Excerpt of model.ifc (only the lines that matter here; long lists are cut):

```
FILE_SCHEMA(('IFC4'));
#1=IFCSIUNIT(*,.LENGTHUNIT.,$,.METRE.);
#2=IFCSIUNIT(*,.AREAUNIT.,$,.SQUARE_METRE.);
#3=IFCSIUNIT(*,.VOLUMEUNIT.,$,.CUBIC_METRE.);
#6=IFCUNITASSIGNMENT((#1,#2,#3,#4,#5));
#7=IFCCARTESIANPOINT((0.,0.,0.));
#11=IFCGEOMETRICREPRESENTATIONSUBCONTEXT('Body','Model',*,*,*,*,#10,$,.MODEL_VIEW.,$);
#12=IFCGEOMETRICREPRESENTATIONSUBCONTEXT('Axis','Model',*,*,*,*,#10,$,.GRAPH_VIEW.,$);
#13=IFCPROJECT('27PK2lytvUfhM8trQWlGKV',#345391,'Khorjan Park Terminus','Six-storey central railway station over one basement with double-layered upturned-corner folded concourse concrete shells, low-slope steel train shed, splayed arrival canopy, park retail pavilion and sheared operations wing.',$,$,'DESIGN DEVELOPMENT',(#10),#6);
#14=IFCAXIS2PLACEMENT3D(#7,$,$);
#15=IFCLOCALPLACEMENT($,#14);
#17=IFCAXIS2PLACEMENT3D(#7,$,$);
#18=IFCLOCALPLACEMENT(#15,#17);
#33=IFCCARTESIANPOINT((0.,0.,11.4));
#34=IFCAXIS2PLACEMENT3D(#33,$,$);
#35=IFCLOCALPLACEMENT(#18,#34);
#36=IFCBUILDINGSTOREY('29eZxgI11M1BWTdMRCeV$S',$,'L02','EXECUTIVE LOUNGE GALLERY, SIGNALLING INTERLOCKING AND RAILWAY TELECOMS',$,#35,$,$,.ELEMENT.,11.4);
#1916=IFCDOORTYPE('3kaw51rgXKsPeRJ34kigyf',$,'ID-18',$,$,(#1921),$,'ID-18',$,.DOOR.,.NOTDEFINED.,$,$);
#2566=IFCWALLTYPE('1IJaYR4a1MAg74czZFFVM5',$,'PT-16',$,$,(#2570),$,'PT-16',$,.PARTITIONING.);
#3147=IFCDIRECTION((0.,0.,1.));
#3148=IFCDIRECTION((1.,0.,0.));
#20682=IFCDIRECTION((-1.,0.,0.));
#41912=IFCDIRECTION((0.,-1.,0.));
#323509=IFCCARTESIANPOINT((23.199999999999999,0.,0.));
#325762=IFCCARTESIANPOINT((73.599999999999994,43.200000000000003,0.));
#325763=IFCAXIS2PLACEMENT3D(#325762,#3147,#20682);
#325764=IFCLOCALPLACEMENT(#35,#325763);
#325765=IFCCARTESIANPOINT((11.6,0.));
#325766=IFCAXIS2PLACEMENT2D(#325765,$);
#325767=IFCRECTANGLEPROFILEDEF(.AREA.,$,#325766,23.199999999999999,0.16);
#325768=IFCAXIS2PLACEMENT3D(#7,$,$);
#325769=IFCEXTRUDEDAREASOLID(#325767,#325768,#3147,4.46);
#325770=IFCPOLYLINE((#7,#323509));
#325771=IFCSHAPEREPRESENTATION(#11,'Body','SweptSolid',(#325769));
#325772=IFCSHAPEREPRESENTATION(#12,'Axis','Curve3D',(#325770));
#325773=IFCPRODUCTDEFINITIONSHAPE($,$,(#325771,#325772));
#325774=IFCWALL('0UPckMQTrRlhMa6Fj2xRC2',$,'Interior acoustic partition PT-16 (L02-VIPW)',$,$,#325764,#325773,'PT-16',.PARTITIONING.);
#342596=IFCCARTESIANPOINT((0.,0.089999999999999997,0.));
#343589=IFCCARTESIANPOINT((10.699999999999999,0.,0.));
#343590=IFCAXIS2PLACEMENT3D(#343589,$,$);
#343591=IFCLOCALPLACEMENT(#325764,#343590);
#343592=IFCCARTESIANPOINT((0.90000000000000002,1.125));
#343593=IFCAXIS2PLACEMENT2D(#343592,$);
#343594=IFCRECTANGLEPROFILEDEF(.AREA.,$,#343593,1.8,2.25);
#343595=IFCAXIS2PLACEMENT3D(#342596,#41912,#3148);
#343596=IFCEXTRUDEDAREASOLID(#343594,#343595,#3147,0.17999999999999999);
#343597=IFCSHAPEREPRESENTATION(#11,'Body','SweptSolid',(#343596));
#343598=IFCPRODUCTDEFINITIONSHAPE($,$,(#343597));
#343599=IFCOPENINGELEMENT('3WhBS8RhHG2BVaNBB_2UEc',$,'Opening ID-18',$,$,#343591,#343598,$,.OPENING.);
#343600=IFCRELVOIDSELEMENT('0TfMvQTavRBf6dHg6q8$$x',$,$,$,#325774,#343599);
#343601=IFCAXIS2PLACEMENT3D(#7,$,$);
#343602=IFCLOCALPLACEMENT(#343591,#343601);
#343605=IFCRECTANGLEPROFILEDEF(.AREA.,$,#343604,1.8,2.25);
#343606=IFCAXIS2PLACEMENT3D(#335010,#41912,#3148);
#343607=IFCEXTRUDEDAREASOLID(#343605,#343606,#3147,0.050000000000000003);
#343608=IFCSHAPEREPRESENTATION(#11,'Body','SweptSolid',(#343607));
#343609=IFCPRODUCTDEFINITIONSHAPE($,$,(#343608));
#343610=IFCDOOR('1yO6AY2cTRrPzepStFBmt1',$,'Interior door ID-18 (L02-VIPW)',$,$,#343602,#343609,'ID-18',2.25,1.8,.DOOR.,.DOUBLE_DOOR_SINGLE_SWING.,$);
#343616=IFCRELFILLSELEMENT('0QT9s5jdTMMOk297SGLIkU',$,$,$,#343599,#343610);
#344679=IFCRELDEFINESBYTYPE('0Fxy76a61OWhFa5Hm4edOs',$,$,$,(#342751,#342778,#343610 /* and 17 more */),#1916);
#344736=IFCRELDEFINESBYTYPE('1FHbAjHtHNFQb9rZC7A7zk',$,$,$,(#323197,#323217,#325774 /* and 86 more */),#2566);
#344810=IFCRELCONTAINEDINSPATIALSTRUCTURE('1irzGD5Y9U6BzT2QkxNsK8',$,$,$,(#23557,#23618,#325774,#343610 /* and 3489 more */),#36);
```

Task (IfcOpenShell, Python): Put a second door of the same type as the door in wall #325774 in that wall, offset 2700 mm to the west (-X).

```python
import ifcopenshell
import ifcopenshell.api.feature
import ifcopenshell.api.geometry
import ifcopenshell.api.root
import ifcopenshell.geom
import ifcopenshell.util.element
import ifcopenshell.util.placement
import ifcopenshell.util.shape
import ifcopenshell.util.unit

model = ifcopenshell.open("model.ifc")
unit_scale = ifcopenshell.util.unit.calculate_unit_scale(model)
settings = ifcopenshell.geom.settings()


def volume(element):
    """Net volume in cubic metres, openings subtracted."""
    shape = ifcopenshell.geom.create_shape(settings, element)
    return ifcopenshell.util.shape.get_volume(shape.geometry)


door = model.by_guid("1yO6AY2cTRrPzepStFBmt1")
opening = door.FillsVoids[0].RelatingOpeningElement
wall = opening.VoidsElements[0].RelatingBuildingElement
before = volume(wall)
shift = ifcopenshell.util.placement.get_local_placement(wall.ObjectPlacement)[:3, 0] * 2.7 / unit_scale

# copy_class copies the void relationship, type, container and properties, but no geometry.
new_opening = ifcopenshell.api.root.copy_class(model, product=opening)
new_opening.Representation = ifcopenshell.util.element.copy_deep(
    model, opening.Representation, exclude=["IfcGeometricRepresentationContext", "IfcRepresentationMap"]
)
new_door = ifcopenshell.api.root.copy_class(model, product=door)
new_door.Representation = ifcopenshell.util.element.copy_deep(
    model, door.Representation, exclude=["IfcGeometricRepresentationContext", "IfcRepresentationMap"]
)
new_door.Tag = None
ifcopenshell.api.feature.add_filling(model, opening=new_opening, element=new_door)

for old, new in ((opening, new_opening), (door, new_door)):
    matrix = ifcopenshell.util.placement.get_local_placement(old.ObjectPlacement)
    matrix[:3, 3] += shift
    ifcopenshell.api.geometry.edit_object_placement(model, product=new, matrix=matrix, is_si=False)

after = volume(wall)

print(f"wall volume {before:.3f} -> {after:.3f} m3")

model.write("model_edited.ifc")
```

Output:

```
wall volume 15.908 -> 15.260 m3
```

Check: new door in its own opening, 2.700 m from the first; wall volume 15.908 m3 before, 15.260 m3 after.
